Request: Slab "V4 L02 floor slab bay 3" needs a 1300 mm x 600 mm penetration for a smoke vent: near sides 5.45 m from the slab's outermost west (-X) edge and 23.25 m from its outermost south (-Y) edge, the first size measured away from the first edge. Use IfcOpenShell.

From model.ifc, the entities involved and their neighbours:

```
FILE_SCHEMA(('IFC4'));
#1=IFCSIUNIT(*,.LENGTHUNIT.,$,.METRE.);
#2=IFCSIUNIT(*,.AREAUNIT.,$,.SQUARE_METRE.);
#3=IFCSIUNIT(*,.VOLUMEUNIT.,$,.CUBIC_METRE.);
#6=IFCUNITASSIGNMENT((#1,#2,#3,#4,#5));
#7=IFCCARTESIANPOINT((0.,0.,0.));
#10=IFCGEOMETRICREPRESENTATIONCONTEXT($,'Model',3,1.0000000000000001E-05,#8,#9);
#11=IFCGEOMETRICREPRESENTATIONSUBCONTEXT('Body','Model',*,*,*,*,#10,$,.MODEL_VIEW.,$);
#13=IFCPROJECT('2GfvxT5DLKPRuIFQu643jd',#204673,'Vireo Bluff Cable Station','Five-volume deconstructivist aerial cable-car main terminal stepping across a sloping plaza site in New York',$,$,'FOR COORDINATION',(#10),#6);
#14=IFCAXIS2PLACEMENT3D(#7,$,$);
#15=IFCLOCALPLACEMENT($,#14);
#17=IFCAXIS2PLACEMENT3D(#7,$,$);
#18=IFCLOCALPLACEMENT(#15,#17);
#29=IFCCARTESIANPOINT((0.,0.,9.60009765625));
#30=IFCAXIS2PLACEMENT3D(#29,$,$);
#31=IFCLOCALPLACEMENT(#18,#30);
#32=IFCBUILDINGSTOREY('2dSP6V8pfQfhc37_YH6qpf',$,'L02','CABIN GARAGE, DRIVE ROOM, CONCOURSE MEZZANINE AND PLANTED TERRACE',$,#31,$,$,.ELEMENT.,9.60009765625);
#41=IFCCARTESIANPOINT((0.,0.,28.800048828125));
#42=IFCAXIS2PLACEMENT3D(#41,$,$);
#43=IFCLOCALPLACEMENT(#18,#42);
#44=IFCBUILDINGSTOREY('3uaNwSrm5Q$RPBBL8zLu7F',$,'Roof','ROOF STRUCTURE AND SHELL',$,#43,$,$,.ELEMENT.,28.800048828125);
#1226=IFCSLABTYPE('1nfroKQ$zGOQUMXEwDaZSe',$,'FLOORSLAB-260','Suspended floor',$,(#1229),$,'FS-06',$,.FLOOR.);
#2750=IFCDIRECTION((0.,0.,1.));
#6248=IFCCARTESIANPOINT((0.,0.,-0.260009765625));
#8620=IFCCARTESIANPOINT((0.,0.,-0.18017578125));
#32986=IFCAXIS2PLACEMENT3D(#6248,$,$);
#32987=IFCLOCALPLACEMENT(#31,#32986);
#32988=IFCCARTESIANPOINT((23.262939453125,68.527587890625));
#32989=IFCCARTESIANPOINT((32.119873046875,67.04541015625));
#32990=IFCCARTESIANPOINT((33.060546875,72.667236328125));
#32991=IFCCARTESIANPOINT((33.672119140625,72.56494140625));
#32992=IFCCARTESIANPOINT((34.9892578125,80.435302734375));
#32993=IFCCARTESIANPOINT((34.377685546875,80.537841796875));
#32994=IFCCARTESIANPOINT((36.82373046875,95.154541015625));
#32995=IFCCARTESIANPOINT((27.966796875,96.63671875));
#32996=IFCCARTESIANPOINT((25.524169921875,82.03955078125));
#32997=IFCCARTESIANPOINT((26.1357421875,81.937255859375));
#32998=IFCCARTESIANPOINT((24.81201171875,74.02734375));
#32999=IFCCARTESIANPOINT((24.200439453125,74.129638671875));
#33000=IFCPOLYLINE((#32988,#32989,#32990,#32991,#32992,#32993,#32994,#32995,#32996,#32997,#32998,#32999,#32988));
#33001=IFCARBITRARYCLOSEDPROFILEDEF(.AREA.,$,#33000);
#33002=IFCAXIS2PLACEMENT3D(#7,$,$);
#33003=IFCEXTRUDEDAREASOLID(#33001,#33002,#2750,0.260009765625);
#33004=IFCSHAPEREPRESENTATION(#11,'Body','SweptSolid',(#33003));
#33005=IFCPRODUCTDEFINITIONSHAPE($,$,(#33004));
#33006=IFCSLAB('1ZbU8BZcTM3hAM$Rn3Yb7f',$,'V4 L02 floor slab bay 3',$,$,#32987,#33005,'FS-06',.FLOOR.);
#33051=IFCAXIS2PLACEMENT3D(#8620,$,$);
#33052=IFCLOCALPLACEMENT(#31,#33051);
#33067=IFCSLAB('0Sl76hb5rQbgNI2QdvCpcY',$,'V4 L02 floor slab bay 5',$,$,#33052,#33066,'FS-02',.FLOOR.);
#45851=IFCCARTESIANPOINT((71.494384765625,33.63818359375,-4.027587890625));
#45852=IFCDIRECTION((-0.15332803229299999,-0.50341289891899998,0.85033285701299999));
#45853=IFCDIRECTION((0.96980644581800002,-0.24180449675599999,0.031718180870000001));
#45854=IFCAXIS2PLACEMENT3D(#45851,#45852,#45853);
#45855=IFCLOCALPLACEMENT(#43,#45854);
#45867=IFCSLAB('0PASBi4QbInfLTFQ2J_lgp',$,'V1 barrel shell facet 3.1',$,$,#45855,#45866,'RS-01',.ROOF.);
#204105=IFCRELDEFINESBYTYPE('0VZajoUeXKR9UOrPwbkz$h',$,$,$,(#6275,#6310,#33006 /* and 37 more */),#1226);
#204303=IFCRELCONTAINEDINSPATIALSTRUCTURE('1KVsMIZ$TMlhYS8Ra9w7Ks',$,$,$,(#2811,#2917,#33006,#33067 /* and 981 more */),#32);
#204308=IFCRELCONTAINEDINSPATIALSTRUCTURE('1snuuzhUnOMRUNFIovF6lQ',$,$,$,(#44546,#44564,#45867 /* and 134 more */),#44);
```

```python
import numpy as np
import ifcopenshell
import ifcopenshell.api.feature
import ifcopenshell.api.geometry
import ifcopenshell.api.root
import ifcopenshell.geom
import ifcopenshell.util.placement
import ifcopenshell.util.representation
import ifcopenshell.util.shape
import ifcopenshell.util.unit

model = ifcopenshell.open("model.ifc")
unit_scale = ifcopenshell.util.unit.calculate_unit_scale(model)
settings = ifcopenshell.geom.settings()


def volume(element):
    """Net volume in cubic metres, openings subtracted."""
    shape = ifcopenshell.geom.create_shape(settings, element)
    return ifcopenshell.util.shape.get_volume(shape.geometry)


slab = model.by_id(33006)
before = volume(slab)

# Extent in the slab's own axes, in metres. The edges named are its -X and -Y sides.
slab_shape = ifcopenshell.geom.create_shape(settings, slab)
vertices = ifcopenshell.util.shape.get_vertices(slab_shape.geometry)
x_min, y_min, bottom = vertices.min(axis=0)
top = vertices[:, 2].max()

opening = ifcopenshell.api.root.create_entity(model, ifc_class="IfcOpeningElement", name="Smoke vent opening", predefined_type="OPENING")
context = ifcopenshell.util.representation.get_context(model, "Model", "Body", "MODEL_VIEW")
width, depth = 1.3, 0.6
outline = [(0.0, 0.0), (width, 0.0), (width, depth), (0.0, depth), (0.0, 0.0)]
# Overshoot both faces by 50 mm so the cut is clean.
shape = ifcopenshell.api.geometry.add_slab_representation(
    model, context=context, depth=top - bottom + 0.1, polyline=outline
)
ifcopenshell.api.geometry.assign_representation(model, product=opening, representation=shape)

matrix = ifcopenshell.util.placement.get_local_placement(slab.ObjectPlacement)
matrix[:, 3] = matrix @ np.append(np.array([x_min + 5.45, y_min + 23.25, bottom - 0.05]) / unit_scale, 1.0)
ifcopenshell.api.geometry.edit_object_placement(model, product=opening, matrix=matrix, is_si=False)
ifcopenshell.api.feature.add_feature(model, feature=opening, element=slab)

after = volume(slab)

print(f"slab volume {before:.3f} -> {after:.3f} m3")

model.write("model_v2.ifc")
```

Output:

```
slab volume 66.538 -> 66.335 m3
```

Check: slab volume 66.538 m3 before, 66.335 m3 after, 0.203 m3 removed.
